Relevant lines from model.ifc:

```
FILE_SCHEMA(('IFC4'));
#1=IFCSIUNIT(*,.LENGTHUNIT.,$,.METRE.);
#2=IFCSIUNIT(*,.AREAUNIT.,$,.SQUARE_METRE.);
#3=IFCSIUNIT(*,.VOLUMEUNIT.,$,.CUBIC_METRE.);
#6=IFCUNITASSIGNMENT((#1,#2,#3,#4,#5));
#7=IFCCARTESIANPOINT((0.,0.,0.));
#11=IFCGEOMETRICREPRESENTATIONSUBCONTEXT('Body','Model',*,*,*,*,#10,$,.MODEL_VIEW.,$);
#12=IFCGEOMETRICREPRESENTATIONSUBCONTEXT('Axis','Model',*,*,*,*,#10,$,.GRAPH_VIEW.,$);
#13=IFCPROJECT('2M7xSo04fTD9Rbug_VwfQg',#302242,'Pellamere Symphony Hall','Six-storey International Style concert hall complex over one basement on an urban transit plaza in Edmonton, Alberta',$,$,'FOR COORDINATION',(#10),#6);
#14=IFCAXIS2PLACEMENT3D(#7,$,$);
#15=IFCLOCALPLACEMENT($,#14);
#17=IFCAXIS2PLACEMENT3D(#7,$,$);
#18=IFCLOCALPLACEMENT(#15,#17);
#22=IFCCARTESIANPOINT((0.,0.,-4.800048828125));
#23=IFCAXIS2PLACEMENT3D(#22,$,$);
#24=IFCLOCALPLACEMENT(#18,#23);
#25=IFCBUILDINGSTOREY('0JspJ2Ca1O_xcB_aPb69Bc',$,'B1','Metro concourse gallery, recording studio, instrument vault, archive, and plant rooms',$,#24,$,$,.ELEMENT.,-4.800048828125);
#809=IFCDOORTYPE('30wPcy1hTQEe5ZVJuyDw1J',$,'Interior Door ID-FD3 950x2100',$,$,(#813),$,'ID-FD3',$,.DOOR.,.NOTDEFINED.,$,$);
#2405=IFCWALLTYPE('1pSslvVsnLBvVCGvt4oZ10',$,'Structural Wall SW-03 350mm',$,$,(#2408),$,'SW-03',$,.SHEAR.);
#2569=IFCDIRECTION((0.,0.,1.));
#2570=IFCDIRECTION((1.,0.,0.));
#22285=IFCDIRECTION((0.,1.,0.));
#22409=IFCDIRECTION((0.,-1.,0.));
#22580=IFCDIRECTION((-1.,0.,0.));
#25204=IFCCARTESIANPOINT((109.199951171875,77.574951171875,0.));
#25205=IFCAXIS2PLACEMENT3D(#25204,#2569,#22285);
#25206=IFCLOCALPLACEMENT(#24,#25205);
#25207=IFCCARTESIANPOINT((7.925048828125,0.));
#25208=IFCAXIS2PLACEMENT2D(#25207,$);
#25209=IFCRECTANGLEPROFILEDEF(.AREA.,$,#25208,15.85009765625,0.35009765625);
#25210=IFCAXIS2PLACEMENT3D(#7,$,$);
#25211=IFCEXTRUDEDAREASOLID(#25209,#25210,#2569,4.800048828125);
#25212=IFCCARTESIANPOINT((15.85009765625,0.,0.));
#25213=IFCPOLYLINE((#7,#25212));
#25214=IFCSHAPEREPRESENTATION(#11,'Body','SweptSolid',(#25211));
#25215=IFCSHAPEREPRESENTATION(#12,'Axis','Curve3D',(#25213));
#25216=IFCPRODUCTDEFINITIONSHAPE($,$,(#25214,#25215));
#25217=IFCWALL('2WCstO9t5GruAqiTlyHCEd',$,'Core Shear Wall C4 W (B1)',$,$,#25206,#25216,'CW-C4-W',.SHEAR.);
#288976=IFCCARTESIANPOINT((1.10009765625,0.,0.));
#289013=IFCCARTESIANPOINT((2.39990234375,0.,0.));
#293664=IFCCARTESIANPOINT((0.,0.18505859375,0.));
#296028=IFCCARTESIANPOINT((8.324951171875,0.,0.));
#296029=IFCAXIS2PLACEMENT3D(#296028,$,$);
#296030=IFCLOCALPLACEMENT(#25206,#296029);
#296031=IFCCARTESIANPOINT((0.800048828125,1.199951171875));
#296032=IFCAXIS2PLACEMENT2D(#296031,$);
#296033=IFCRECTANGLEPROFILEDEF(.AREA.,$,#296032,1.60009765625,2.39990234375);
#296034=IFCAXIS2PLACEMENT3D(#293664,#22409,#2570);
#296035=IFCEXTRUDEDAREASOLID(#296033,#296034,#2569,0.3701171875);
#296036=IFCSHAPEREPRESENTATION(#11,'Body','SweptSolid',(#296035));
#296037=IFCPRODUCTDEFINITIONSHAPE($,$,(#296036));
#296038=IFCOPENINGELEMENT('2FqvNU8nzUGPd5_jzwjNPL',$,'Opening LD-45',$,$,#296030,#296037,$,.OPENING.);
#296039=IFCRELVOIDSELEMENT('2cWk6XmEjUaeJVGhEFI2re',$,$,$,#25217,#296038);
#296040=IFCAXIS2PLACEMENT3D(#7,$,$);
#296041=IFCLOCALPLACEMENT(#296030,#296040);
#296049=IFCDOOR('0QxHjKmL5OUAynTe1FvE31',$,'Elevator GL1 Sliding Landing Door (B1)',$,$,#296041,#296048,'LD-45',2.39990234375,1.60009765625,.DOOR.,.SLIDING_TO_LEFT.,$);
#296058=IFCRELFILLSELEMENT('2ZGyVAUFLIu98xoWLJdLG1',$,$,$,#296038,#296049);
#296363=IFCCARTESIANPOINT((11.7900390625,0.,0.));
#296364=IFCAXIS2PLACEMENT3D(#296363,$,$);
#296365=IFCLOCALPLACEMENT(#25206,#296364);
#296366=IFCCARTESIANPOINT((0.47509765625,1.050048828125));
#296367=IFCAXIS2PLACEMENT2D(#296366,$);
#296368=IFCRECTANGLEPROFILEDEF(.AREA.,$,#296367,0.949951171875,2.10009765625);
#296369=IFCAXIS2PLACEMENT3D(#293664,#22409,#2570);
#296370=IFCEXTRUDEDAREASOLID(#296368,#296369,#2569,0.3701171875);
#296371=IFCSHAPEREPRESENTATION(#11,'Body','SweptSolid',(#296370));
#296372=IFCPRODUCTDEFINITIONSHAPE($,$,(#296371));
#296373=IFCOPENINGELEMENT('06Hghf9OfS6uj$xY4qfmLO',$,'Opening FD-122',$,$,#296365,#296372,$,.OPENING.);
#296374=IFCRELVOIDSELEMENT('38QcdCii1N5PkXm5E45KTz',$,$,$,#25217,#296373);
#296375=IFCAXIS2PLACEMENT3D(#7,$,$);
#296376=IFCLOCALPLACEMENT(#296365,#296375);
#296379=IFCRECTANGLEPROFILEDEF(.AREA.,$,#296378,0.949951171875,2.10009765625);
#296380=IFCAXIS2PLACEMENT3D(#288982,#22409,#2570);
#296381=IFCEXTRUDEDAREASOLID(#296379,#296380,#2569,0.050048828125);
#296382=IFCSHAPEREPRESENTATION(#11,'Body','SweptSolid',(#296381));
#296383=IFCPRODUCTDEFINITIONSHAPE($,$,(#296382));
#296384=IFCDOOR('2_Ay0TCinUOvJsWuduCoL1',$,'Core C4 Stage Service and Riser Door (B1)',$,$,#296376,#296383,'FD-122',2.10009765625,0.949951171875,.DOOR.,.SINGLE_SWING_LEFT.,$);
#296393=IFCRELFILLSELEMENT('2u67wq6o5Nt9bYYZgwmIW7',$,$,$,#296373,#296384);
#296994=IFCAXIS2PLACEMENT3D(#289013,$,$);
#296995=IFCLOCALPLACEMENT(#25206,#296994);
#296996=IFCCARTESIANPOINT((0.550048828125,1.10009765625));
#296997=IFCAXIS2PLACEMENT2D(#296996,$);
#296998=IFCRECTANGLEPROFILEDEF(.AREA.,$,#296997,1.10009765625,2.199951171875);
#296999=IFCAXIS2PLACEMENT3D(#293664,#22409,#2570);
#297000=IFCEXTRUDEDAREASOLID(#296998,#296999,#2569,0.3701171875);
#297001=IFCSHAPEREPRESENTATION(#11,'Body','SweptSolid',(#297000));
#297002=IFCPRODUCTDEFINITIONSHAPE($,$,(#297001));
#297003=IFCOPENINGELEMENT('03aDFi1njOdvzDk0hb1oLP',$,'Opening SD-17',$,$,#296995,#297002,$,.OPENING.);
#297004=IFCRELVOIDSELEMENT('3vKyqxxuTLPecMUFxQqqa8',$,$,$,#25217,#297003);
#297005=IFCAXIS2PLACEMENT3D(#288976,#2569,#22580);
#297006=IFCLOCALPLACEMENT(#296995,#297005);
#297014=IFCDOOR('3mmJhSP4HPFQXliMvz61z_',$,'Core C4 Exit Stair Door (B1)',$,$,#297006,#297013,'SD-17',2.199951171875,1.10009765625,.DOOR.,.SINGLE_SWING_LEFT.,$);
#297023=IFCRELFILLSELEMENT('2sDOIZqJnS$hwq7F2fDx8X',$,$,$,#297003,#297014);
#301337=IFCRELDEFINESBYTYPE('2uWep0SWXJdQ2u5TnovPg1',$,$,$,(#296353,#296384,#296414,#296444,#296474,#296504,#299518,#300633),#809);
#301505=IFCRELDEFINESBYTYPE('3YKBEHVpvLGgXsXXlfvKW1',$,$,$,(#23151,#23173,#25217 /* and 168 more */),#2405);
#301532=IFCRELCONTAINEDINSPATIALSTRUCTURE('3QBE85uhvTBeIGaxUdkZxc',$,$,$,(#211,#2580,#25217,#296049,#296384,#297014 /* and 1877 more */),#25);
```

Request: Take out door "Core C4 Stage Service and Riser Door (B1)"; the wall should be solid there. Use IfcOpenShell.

```python
import ifcopenshell
import ifcopenshell.api.feature
import ifcopenshell.api.root
import ifcopenshell.geom
import ifcopenshell.util.shape

model = ifcopenshell.open("model.ifc")
settings = ifcopenshell.geom.settings()


def volume(element):
    """Net volume in cubic metres, openings subtracted."""
    shape = ifcopenshell.geom.create_shape(settings, element)
    return ifcopenshell.util.shape.get_volume(shape.geometry)


door = model.by_guid("2_Ay0TCinUOvJsWuduCoL1")
opening = door.FillsVoids[0].RelatingOpeningElement
wall = opening.VoidsElements[0].RelatingBuildingElement
before = volume(wall)

ifcopenshell.api.root.remove_product(model, product=door)
ifcopenshell.api.feature.remove_feature(model, feature=opening)

after = volume(wall)

print(f"wall volume {before:.3f} -> {after:.3f} m3")

model.write("model-out.ifc")
```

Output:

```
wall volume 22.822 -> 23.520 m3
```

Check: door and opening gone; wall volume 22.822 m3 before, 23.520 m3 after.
